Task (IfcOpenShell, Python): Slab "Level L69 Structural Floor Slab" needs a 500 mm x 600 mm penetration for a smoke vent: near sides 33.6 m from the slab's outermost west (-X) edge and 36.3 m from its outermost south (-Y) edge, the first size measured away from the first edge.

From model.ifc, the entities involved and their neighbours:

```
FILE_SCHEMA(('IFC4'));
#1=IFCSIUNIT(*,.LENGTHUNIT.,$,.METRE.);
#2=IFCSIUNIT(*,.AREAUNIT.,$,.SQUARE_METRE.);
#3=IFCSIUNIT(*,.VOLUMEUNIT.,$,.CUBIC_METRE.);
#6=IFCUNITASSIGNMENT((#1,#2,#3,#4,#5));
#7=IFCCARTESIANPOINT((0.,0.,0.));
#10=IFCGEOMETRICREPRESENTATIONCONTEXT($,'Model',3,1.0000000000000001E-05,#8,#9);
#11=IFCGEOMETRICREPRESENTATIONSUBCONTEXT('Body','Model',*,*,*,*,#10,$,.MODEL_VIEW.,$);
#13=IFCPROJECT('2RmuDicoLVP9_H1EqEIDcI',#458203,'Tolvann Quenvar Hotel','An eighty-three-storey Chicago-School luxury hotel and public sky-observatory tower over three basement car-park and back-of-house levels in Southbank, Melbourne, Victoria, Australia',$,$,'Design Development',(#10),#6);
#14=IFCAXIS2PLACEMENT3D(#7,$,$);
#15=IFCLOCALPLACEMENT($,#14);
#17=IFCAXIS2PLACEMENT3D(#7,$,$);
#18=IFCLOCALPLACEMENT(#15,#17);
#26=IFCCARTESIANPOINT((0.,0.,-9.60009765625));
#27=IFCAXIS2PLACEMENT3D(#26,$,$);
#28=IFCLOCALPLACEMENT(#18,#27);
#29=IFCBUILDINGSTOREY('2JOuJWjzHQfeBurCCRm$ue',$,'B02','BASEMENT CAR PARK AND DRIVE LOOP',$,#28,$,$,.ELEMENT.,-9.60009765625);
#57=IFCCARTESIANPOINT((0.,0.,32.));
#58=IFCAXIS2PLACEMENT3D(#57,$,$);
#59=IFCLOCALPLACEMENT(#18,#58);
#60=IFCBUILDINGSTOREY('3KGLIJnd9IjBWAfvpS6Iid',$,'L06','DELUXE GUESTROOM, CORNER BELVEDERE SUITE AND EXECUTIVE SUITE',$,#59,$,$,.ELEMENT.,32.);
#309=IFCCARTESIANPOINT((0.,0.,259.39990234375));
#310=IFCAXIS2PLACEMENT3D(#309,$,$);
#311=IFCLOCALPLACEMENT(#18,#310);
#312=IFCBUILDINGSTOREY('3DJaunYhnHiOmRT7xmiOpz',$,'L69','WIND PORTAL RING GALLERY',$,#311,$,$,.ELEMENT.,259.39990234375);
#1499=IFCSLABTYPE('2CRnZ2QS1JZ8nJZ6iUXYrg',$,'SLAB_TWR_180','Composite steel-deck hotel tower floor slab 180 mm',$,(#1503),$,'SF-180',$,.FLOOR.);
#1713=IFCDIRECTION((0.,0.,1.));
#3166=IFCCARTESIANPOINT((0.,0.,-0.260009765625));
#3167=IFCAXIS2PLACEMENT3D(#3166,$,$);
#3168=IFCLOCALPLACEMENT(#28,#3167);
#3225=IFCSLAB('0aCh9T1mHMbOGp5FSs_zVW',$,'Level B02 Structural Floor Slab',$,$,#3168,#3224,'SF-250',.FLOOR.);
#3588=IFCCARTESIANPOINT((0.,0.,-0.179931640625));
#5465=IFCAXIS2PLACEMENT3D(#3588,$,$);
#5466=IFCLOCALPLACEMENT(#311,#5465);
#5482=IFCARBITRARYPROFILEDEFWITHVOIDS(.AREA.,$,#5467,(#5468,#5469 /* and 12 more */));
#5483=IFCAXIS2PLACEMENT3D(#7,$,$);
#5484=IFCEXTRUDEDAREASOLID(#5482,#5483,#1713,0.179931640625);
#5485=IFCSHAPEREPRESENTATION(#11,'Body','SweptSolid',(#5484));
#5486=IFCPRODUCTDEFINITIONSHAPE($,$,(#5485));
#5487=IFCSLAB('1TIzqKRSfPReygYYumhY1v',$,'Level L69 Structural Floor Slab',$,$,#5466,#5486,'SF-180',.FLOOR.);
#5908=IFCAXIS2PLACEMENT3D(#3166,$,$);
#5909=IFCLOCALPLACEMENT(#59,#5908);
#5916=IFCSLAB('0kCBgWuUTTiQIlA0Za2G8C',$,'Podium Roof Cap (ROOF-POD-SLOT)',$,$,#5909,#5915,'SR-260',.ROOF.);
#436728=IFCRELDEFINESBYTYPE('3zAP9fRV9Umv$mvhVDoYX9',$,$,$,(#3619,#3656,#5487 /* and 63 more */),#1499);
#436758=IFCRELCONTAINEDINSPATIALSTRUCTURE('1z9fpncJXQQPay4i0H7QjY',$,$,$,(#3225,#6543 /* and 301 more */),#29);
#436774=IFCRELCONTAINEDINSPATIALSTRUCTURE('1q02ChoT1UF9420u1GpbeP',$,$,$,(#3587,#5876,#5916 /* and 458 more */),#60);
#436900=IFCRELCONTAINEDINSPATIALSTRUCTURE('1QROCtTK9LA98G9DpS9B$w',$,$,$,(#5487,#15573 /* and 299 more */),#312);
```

```python
import numpy as np
import ifcopenshell
import ifcopenshell.api.feature
import ifcopenshell.api.geometry
import ifcopenshell.api.root
import ifcopenshell.geom
import ifcopenshell.util.placement
import ifcopenshell.util.representation
import ifcopenshell.util.shape
import ifcopenshell.util.unit

model = ifcopenshell.open("model.ifc")
unit_scale = ifcopenshell.util.unit.calculate_unit_scale(model)
settings = ifcopenshell.geom.settings()


def volume(element):
    """Net volume in cubic metres, openings subtracted."""
    shape = ifcopenshell.geom.create_shape(settings, element)
    return ifcopenshell.util.shape.get_volume(shape.geometry)


slab = model.by_id(5487)
before = volume(slab)

# Extent in the slab's own axes, in metres. The edges named are its -X and -Y sides.
slab_shape = ifcopenshell.geom.create_shape(settings, slab)
vertices = ifcopenshell.util.shape.get_vertices(slab_shape.geometry)
x_min, y_min, bottom = vertices.min(axis=0)
top = vertices[:, 2].max()

opening = ifcopenshell.api.root.create_entity(model, ifc_class="IfcOpeningElement", name="Smoke vent opening", predefined_type="OPENING")
context = ifcopenshell.util.representation.get_context(model, "Model", "Body", "MODEL_VIEW")
width, depth = 0.5, 0.6
outline = [(0.0, 0.0), (width, 0.0), (width, depth), (0.0, depth), (0.0, 0.0)]
# Overshoot both faces by 50 mm so the cut is clean.
shape = ifcopenshell.api.geometry.add_slab_representation(
    model, context=context, depth=top - bottom + 0.1, polyline=outline
)
ifcopenshell.api.geometry.assign_representation(model, product=opening, representation=shape)

matrix = ifcopenshell.util.placement.get_local_placement(slab.ObjectPlacement)
matrix[:, 3] = matrix @ np.append(np.array([x_min + 33.6, y_min + 36.3, bottom - 0.05]) / unit_scale, 1.0)
ifcopenshell.api.geometry.edit_object_placement(model, product=opening, matrix=matrix, is_si=False)
ifcopenshell.api.feature.add_feature(model, feature=opening, element=slab)

after = volume(slab)

print(f"slab volume {before:.3f} -> {after:.3f} m3")

model.write("model_rev.ifc")
```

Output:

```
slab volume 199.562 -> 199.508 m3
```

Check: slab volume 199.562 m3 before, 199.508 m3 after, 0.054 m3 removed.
